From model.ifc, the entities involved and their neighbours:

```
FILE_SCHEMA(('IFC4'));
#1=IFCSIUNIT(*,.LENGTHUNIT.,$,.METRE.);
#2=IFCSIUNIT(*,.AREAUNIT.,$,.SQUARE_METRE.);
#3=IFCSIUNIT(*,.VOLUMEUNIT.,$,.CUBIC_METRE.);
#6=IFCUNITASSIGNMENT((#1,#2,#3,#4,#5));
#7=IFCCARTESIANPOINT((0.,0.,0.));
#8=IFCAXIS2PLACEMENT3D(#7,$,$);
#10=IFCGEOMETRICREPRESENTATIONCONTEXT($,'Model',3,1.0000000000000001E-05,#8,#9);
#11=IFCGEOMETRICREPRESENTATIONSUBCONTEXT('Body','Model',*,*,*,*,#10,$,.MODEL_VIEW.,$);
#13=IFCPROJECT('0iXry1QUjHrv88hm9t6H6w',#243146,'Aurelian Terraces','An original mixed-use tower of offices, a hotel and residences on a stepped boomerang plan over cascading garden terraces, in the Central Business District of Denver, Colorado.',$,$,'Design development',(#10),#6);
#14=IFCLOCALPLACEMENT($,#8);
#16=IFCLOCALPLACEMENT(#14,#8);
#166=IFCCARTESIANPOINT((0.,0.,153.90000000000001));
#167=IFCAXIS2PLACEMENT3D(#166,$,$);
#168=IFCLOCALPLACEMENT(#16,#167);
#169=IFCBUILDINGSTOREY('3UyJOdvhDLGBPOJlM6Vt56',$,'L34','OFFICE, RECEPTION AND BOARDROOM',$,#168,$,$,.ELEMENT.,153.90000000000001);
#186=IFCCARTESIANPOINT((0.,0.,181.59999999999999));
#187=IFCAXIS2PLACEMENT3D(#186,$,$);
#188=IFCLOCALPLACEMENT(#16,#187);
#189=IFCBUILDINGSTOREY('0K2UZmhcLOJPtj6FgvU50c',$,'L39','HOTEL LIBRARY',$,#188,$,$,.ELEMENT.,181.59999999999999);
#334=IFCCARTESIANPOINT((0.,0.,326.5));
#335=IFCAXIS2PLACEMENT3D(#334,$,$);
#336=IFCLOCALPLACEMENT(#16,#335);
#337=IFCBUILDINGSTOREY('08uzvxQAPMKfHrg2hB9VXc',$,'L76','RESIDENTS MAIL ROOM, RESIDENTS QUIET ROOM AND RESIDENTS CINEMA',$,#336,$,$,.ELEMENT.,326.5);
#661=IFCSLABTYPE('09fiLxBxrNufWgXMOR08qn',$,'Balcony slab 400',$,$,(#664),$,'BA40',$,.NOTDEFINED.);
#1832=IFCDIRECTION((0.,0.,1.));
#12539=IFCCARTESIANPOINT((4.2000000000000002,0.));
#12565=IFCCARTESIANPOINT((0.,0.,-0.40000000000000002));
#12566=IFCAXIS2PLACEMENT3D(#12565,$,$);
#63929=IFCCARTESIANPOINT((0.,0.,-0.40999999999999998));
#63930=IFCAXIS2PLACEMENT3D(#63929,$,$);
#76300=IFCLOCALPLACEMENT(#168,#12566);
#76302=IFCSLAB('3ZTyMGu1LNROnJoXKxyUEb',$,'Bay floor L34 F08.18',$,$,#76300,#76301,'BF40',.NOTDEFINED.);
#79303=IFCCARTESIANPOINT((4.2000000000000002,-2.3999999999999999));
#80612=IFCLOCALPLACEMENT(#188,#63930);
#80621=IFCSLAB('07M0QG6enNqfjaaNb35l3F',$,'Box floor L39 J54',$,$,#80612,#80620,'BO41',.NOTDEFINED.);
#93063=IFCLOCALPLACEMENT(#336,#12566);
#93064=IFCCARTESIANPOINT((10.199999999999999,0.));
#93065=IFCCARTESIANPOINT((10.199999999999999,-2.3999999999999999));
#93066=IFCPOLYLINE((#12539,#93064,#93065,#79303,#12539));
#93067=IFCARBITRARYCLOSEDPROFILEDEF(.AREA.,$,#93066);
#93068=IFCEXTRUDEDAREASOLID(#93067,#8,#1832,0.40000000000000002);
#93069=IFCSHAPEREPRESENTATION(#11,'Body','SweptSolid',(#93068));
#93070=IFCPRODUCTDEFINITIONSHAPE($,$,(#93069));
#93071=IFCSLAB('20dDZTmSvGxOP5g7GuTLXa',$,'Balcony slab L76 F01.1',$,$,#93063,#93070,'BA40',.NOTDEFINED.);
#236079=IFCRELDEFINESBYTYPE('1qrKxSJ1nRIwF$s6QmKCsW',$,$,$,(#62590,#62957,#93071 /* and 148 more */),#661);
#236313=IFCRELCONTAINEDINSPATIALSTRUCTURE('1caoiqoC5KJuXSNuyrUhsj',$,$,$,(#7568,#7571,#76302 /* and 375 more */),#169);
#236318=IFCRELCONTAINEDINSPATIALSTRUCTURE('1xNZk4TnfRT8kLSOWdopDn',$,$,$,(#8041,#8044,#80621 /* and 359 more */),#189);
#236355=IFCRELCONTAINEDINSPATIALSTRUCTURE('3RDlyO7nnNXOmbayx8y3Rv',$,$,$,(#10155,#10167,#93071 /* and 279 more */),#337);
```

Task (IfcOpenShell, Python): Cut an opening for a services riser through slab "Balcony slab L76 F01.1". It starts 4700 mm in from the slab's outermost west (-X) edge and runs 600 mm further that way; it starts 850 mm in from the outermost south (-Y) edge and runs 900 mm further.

```python
import numpy as np
import ifcopenshell
import ifcopenshell.api.feature
import ifcopenshell.api.geometry
import ifcopenshell.api.root
import ifcopenshell.geom
import ifcopenshell.util.placement
import ifcopenshell.util.representation
import ifcopenshell.util.shape
import ifcopenshell.util.unit

model = ifcopenshell.open("model.ifc")
unit_scale = ifcopenshell.util.unit.calculate_unit_scale(model)
settings = ifcopenshell.geom.settings()


def volume(element):
    """Net volume in cubic metres, openings subtracted."""
    shape = ifcopenshell.geom.create_shape(settings, element)
    return ifcopenshell.util.shape.get_volume(shape.geometry)


slab = model.by_id(93071)
before = volume(slab)

# Extent in the slab's own axes, in metres. The edges named are its -X and -Y sides.
slab_shape = ifcopenshell.geom.create_shape(settings, slab)
vertices = ifcopenshell.util.shape.get_vertices(slab_shape.geometry)
x_min, y_min, bottom = vertices.min(axis=0)
top = vertices[:, 2].max()

opening = ifcopenshell.api.root.create_entity(model, ifc_class="IfcOpeningElement", name="Services riser opening", predefined_type="OPENING")
context = ifcopenshell.util.representation.get_context(model, "Model", "Body", "MODEL_VIEW")
width, depth = 0.6, 0.9
outline = [(0.0, 0.0), (width, 0.0), (width, depth), (0.0, depth), (0.0, 0.0)]
# Overshoot both faces by 50 mm so the cut is clean.
shape = ifcopenshell.api.geometry.add_slab_representation(
    model, context=context, depth=top - bottom + 0.1, polyline=outline
)
ifcopenshell.api.geometry.assign_representation(model, product=opening, representation=shape)

matrix = ifcopenshell.util.placement.get_local_placement(slab.ObjectPlacement)
matrix[:, 3] = matrix @ np.append(np.array([x_min + 4.7, y_min + 0.85, bottom - 0.05]) / unit_scale, 1.0)
ifcopenshell.api.geometry.edit_object_placement(model, product=opening, matrix=matrix, is_si=False)
ifcopenshell.api.feature.add_feature(model, feature=opening, element=slab)

after = volume(slab)

print(f"slab volume {before:.3f} -> {after:.3f} m3")

model.write("model_rev.ifc")
```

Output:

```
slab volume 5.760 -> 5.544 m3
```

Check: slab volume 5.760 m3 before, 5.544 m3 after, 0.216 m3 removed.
